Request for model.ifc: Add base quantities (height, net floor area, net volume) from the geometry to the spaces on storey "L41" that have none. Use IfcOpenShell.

First a look at what the model holds.

```python
import ifcopenshell
import ifcopenshell.util.element
import ifcopenshell.util.unit

model = ifcopenshell.open("model.ifc")
print(model.schema)
for unit_type in ("LENGTHUNIT", "AREAUNIT", "VOLUMEUNIT"):
    print(unit_type, ifcopenshell.util.unit.calculate_unit_scale(model, unit_type))
storey = next(s for s in model.by_type("IfcBuildingStorey") if s.Name == "L41")
spaces = [e for e in ifcopenshell.util.element.get_decomposition(storey) if e.is_a("IfcSpace")]
for e in sorted(spaces, key=lambda e: e.id()):
    print(e.id(), e.is_a(), e.Name, list(ifcopenshell.util.element.get_psets(e, qtos_only=True)), sep=" | ")
```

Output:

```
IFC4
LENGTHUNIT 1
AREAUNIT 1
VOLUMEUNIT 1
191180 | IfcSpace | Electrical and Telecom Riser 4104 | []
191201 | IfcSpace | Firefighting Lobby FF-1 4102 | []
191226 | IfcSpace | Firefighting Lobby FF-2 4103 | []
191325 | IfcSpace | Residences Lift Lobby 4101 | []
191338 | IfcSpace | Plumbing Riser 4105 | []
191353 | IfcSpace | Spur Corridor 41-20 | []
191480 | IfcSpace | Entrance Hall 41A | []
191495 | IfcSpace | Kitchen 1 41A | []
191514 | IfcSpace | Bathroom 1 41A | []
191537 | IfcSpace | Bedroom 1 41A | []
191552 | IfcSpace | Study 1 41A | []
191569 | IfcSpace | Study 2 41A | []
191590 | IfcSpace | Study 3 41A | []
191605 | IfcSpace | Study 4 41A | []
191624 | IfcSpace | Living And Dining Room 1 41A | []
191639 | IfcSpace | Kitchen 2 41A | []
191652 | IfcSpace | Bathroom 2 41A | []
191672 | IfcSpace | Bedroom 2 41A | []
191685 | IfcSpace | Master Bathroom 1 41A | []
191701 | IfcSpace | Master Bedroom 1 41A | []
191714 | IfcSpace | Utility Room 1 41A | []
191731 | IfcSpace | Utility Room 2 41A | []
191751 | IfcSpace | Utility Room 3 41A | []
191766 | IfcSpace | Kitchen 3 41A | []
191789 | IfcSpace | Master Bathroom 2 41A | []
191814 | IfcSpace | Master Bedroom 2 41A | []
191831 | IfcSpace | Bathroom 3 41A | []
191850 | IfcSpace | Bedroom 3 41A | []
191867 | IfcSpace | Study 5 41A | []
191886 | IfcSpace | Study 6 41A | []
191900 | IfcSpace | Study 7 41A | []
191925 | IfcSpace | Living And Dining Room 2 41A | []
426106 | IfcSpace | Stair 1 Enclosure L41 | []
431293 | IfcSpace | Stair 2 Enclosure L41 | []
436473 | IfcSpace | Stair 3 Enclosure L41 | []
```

```python
import ifcopenshell
import ifcopenshell.api.pset
import ifcopenshell.geom
import ifcopenshell.util.element
import ifcopenshell.util.shape
import ifcopenshell.util.unit

model = ifcopenshell.open("model.ifc")
unit_scale = ifcopenshell.util.unit.calculate_unit_scale(model)
area_scale = ifcopenshell.util.unit.calculate_unit_scale(model, "AREAUNIT")
volume_scale = ifcopenshell.util.unit.calculate_unit_scale(model, "VOLUMEUNIT")
settings = ifcopenshell.geom.settings()

storey = next(s for s in model.by_type("IfcBuildingStorey") if s.Name == "L41")
spaces = [e for e in ifcopenshell.util.element.get_decomposition(storey) if e.is_a("IfcSpace")]

for e in sorted(spaces, key=lambda e: e.id()):
    if ifcopenshell.util.element.get_psets(e, qtos_only=True, should_inherit=False):
        continue
    # Geometry comes back in metres, in the element's own axes.
    shape = ifcopenshell.geom.create_shape(settings, e)
    values = {
        "Height": ifcopenshell.util.shape.get_z(shape.geometry) / unit_scale,
        "NetFloorArea": ifcopenshell.util.shape.get_footprint_area(shape.geometry) / area_scale,
        "NetVolume": ifcopenshell.util.shape.get_volume(shape.geometry) / volume_scale,
    }
    qto = ifcopenshell.api.pset.add_qto(model, product=e, name="Qto_SpaceBaseQuantities")
    ifcopenshell.api.pset.edit_qto(model, qto=qto, properties=values)
    print(e.id(), {k: round(v, 3) for k, v in values.items()})

model.write("model_updated.ifc")
```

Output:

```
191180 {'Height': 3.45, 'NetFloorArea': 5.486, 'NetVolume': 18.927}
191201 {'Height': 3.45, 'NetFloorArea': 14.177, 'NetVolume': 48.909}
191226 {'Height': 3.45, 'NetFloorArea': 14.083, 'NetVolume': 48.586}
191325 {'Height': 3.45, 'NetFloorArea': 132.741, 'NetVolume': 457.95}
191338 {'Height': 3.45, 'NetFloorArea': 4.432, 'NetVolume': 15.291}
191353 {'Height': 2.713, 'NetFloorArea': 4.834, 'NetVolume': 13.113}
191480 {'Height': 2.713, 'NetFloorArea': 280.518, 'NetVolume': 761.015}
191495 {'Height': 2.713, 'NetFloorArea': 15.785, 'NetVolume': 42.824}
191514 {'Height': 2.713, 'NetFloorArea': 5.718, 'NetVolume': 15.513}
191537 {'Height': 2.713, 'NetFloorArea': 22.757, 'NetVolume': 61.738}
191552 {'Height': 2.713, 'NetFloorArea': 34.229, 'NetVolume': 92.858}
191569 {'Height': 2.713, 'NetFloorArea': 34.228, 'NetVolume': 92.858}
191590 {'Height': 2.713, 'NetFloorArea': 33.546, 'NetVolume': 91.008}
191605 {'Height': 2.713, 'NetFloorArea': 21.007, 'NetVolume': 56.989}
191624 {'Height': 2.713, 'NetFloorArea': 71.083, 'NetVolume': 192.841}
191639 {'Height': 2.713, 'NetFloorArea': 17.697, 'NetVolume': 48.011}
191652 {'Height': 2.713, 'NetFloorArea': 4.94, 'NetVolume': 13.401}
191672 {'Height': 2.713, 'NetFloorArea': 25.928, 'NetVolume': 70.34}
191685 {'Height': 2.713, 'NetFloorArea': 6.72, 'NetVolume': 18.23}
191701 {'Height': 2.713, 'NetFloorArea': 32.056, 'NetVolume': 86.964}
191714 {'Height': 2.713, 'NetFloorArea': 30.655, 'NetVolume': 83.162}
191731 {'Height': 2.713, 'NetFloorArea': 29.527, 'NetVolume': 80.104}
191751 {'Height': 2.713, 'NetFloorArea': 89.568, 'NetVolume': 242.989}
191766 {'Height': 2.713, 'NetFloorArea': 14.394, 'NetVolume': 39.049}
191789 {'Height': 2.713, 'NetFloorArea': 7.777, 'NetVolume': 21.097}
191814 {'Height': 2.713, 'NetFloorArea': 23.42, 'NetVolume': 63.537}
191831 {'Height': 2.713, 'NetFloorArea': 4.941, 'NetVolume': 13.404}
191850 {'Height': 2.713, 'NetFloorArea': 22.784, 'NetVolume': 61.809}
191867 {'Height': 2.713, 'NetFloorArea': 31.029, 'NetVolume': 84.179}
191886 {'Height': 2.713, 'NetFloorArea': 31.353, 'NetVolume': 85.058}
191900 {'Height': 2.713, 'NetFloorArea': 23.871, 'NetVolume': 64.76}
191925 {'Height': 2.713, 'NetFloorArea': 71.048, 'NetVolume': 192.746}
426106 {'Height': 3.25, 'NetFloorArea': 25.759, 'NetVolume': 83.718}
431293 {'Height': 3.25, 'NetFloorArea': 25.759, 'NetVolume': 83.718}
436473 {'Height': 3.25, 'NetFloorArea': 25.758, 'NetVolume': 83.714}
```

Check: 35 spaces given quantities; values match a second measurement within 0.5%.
